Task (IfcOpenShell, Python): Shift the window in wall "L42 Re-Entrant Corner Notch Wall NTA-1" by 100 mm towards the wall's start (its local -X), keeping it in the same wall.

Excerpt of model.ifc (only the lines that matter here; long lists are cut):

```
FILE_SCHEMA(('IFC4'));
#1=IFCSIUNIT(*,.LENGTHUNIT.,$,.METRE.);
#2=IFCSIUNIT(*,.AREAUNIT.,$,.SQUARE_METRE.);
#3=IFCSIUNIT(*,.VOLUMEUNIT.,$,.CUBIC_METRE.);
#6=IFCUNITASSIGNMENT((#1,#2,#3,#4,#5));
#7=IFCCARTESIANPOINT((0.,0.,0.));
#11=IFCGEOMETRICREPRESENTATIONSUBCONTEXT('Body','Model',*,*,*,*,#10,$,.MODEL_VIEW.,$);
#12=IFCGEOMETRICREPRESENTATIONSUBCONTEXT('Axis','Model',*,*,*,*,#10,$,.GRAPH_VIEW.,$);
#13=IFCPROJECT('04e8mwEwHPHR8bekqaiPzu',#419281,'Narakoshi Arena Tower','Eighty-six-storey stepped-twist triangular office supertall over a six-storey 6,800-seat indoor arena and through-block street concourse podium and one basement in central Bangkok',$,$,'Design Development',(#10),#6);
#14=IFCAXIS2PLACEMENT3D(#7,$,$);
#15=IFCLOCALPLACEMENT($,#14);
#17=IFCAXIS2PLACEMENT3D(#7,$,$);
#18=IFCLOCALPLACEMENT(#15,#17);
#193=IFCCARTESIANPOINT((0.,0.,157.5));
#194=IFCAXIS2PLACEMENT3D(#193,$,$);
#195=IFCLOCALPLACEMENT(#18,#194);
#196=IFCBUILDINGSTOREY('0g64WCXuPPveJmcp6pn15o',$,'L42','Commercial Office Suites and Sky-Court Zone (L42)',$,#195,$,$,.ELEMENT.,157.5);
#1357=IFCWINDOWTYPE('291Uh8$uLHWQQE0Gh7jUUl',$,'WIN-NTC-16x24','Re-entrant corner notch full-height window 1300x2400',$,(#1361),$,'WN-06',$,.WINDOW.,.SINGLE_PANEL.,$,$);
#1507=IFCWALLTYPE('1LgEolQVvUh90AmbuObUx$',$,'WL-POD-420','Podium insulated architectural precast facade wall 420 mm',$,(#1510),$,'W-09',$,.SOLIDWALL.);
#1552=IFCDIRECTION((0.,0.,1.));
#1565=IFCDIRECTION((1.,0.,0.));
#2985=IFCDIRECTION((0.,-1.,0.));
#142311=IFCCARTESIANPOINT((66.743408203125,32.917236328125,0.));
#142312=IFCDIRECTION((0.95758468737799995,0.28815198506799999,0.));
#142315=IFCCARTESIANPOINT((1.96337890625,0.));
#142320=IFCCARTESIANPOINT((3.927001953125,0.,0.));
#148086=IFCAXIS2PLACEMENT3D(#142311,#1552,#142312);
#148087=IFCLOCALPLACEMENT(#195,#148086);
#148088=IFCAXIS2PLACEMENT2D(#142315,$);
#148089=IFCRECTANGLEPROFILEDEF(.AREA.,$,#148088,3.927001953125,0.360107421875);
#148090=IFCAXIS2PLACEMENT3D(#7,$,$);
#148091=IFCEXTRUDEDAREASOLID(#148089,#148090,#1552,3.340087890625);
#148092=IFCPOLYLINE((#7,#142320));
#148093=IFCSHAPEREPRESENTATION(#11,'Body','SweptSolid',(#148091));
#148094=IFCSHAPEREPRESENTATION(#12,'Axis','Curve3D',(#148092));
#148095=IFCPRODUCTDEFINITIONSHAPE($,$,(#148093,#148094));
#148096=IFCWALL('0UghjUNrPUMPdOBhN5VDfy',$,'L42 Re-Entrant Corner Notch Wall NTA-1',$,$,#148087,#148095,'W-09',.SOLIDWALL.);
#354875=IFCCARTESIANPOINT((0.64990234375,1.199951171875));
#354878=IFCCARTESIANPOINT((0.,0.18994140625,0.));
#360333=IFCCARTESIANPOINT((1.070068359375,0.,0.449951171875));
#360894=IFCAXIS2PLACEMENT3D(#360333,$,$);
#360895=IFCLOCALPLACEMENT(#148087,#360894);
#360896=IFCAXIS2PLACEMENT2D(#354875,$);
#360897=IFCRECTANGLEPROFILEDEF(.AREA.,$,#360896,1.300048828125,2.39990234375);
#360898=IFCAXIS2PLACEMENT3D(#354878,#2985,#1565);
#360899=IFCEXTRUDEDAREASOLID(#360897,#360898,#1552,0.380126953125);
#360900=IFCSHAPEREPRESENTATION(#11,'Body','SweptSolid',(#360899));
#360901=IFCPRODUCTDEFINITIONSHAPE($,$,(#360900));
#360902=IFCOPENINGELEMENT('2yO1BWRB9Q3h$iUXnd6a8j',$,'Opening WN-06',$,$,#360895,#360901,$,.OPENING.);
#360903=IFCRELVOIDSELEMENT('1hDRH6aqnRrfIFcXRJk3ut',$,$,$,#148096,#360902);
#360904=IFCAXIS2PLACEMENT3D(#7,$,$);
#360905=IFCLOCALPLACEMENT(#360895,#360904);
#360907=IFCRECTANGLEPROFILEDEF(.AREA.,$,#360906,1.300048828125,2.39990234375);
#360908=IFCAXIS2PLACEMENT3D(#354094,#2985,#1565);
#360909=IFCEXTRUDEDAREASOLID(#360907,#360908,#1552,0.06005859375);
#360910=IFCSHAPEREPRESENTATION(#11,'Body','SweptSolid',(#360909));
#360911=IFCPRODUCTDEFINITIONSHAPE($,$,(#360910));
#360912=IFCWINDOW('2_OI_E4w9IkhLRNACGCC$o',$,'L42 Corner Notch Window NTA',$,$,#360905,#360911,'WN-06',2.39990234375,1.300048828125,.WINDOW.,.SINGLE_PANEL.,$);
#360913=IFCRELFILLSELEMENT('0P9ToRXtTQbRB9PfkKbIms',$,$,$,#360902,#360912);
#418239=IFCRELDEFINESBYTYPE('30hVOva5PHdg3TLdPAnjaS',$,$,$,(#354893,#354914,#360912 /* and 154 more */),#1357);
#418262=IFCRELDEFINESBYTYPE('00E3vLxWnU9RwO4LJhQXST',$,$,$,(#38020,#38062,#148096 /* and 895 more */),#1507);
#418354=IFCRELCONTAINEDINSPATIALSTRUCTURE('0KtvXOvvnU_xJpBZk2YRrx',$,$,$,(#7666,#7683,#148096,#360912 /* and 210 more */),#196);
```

```python
import ifcopenshell
import ifcopenshell.api.geometry
import ifcopenshell.util.placement
import ifcopenshell.util.unit

model = ifcopenshell.open("model.ifc")
unit_scale = ifcopenshell.util.unit.calculate_unit_scale(model)

window = model.by_guid("2_OI_E4w9IkhLRNACGCC$o")
opening = window.FillsVoids[0].RelatingOpeningElement
wall = opening.VoidsElements[0].RelatingBuildingElement

wall_matrix = ifcopenshell.util.placement.get_local_placement(wall.ObjectPlacement)
shift = wall_matrix[:3, 0] * -0.1 / unit_scale
before = ifcopenshell.util.placement.get_local_placement(window.ObjectPlacement)[:3, 3].copy()

# The window is placed relative to its opening, so it follows when the opening moves.
matrix = ifcopenshell.util.placement.get_local_placement(opening.ObjectPlacement)
matrix[:3, 3] += shift
ifcopenshell.api.geometry.edit_object_placement(
    model, product=opening, matrix=matrix, is_si=False, should_transform_children=True
)

after = ifcopenshell.util.placement.get_local_placement(window.ObjectPlacement)[:3, 3]
print("window moved by", (after - before).round(3) + 0.0)

model.write("model_rev.ifc")
```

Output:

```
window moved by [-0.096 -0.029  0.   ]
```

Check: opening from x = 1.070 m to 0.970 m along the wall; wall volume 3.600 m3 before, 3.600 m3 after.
